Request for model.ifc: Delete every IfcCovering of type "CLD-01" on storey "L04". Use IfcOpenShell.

First a look at what the model holds.

```python
import ifcopenshell
import ifcopenshell.util.element

model = ifcopenshell.open("model.ifc")
print(model.schema)
storey = next(s for s in model.by_type("IfcBuildingStorey") if s.Name == "L04")
coverings = [e for e in ifcopenshell.util.element.get_decomposition(storey) if e.is_a("IfcCovering")]
seen = {}
for e in coverings:
    element_type = ifcopenshell.util.element.get_type(e)
    name = element_type.Name if element_type not in (None, e) else None
    seen[name] = seen.get(name, 0) + 1
for name, count in sorted(seen.items(), key=str):
    print(count, "x", name)
```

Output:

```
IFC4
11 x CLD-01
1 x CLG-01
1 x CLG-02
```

```python
import ifcopenshell
import ifcopenshell.api.root
import ifcopenshell.util.element

model = ifcopenshell.open("model.ifc")

storey = next(s for s in model.by_type("IfcBuildingStorey") if s.Name == "L04")
coverings = [e for e in ifcopenshell.util.element.get_decomposition(storey) if e.is_a("IfcCovering")]
targets = [e for e in coverings if (t := ifcopenshell.util.element.get_type(e)) not in (None, e) and t.Name == "CLD-01"]

for e in targets:
    ifcopenshell.api.root.remove_product(model, product=e)
print(len(targets), "removed")

model.write("model_v2.ifc")
```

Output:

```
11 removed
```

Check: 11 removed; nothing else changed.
